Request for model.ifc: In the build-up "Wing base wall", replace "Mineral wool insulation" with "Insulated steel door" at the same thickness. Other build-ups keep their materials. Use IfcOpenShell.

First a look at what the model holds.

```python
import ifcopenshell
import ifcopenshell.util.element

model = ifcopenshell.open("model.ifc")
print(model.schema)
for layer_set in model.by_type("IfcMaterialLayerSet"):
    if layer_set.LayerSetName == "Wing base wall":
        for layer in layer_set.MaterialLayers:
            print(layer.id(), layer.Material and layer.Material.Name, layer.LayerThickness, sep=" | ")
        print(len(ifcopenshell.util.element.get_elements_by_material(model, layer_set)), "elements and types use it")
print(sorted(m.Name for m in model.by_type("IfcMaterial") if m.Name)[:60])
```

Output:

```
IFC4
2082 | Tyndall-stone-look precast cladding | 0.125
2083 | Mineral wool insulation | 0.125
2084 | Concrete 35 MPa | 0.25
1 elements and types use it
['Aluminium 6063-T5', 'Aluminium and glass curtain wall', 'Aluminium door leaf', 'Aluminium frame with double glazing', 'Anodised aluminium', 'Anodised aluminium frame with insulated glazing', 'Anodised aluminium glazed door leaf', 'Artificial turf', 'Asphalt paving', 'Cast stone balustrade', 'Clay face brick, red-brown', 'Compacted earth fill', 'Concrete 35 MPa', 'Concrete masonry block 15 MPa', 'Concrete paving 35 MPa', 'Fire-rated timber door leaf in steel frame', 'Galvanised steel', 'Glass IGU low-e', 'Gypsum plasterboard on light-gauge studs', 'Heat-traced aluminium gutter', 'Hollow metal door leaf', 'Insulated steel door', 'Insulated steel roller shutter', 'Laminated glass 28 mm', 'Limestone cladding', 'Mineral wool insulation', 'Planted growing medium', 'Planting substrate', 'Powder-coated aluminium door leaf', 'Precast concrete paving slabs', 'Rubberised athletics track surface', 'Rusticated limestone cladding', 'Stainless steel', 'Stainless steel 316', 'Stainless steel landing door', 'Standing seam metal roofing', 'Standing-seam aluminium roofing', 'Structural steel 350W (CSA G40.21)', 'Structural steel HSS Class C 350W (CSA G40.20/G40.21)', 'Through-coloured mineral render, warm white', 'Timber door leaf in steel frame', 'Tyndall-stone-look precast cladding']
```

```python
import ifcopenshell
import ifcopenshell.api.material

model = ifcopenshell.open("model.ifc")

layer_set = next(s for s in model.by_type("IfcMaterialLayerSet") if s.LayerSetName == "Wing base wall")
layer = next(l for l in layer_set.MaterialLayers if l.Material and l.Material.Name == "Mineral wool insulation")
material = next(m for m in model.by_type("IfcMaterial") if m.Name == "Insulated steel door")

# Point this one layer at the other material; renaming the old one would change it everywhere.
ifcopenshell.api.material.edit_layer(model, layer=layer, attributes={"Name": material.Name}, material=material)

print([l.Material.Name if l.Material else None for l in layer_set.MaterialLayers])

model.write("model_v2.ifc")
```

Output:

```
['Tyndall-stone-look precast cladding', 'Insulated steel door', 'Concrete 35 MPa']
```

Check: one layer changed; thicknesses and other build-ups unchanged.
